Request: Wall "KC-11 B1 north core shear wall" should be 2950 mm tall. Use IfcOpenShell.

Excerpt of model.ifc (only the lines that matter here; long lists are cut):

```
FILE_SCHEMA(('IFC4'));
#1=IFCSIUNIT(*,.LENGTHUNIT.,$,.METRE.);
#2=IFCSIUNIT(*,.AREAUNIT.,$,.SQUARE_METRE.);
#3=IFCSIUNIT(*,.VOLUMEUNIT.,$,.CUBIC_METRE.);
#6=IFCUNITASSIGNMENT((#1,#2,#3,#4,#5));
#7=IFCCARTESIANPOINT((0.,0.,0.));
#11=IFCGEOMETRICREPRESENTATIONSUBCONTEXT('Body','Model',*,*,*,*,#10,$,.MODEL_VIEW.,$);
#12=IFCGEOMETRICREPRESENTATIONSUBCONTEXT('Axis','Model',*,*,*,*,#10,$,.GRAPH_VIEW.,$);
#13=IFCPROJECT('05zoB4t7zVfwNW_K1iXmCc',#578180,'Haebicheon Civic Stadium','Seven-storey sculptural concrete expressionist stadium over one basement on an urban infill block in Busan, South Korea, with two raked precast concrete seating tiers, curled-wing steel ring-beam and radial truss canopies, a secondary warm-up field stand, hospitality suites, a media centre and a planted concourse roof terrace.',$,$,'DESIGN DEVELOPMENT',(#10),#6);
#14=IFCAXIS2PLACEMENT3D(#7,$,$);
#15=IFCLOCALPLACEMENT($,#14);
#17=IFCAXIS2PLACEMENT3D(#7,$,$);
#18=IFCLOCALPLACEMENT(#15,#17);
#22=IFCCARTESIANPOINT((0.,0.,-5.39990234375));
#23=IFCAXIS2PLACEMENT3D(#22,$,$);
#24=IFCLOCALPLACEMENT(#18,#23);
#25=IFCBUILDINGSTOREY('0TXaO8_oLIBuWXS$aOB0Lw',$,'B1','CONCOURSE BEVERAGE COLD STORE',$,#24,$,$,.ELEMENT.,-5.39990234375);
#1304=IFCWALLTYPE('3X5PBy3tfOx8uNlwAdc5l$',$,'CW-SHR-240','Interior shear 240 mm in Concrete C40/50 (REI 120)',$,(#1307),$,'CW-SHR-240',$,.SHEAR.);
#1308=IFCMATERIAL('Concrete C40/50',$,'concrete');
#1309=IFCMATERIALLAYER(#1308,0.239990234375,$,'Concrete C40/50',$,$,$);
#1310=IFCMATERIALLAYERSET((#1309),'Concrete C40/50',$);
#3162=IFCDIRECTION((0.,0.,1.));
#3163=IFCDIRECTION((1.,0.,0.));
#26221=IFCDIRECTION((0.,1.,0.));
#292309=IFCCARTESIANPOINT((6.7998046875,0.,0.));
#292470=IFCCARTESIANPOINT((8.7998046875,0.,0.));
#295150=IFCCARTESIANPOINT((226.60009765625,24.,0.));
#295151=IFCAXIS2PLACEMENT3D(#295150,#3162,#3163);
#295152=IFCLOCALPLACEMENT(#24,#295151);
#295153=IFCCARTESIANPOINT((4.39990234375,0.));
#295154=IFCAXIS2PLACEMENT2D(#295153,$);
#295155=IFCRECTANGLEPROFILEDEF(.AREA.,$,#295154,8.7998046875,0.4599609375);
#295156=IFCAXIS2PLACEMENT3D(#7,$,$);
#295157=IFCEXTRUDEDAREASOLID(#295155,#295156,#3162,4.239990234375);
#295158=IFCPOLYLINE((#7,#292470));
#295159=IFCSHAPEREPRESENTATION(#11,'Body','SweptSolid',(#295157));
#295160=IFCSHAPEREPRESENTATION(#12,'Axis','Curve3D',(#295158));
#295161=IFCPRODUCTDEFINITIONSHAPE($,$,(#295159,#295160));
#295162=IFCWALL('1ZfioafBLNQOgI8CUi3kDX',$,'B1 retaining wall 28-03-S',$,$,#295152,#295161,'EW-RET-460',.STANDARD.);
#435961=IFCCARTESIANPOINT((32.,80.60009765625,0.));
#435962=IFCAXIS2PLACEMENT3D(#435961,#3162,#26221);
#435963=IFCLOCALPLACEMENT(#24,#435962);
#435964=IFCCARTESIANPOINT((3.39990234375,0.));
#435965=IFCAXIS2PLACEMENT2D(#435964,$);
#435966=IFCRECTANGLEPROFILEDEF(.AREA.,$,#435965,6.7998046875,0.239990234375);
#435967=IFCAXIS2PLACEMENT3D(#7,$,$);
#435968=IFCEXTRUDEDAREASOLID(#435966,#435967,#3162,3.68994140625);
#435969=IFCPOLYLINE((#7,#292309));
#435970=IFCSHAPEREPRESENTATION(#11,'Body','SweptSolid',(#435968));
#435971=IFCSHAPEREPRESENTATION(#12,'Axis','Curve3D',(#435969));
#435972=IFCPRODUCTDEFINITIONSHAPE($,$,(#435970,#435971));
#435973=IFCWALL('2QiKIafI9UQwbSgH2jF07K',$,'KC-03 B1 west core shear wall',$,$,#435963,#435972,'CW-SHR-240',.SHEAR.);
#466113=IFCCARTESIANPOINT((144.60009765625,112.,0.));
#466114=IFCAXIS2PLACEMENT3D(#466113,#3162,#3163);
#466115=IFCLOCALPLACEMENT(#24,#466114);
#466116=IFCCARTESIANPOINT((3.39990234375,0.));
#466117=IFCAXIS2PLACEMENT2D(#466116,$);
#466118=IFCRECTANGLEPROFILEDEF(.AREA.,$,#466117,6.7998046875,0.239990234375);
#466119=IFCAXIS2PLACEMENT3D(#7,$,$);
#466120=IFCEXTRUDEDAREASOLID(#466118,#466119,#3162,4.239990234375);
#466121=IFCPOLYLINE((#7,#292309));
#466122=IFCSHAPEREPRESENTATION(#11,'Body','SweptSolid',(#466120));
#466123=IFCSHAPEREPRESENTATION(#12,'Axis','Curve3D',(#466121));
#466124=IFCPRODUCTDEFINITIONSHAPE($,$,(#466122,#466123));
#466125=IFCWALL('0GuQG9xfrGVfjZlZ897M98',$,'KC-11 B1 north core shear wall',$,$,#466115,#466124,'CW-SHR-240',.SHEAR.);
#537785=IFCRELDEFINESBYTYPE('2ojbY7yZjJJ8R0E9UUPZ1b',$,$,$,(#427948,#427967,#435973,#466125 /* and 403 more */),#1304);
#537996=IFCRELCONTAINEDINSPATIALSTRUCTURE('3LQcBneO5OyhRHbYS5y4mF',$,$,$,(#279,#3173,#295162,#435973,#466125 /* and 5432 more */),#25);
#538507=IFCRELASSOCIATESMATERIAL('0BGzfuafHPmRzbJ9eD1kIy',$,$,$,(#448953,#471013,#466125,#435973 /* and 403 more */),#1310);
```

```python
import ifcopenshell
import ifcopenshell.geom
import ifcopenshell.util.representation
import ifcopenshell.util.shape
import ifcopenshell.util.unit

model = ifcopenshell.open("model.ifc")
unit_scale = ifcopenshell.util.unit.calculate_unit_scale(model)
settings = ifcopenshell.geom.settings()


def volume(element):
    """Net volume in cubic metres, openings subtracted."""
    shape = ifcopenshell.geom.create_shape(settings, element)
    return ifcopenshell.util.shape.get_volume(shape.geometry)


wall = model.by_guid("0GuQG9xfrGVfjZlZ897M98")
before = volume(wall)

body = ifcopenshell.util.representation.get_representation(wall, "Model", "Body")
solid = body.Items[0]
old_height = solid.Depth
solid.Depth = 2.95 / unit_scale
after = volume(wall)

print(f"height {old_height:g} -> {solid.Depth:g}, volume {before:.3f} -> {after:.3f} m3")

model.write("model-out.ifc")
```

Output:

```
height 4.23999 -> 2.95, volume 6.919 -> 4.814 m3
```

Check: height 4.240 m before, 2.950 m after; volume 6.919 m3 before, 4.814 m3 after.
